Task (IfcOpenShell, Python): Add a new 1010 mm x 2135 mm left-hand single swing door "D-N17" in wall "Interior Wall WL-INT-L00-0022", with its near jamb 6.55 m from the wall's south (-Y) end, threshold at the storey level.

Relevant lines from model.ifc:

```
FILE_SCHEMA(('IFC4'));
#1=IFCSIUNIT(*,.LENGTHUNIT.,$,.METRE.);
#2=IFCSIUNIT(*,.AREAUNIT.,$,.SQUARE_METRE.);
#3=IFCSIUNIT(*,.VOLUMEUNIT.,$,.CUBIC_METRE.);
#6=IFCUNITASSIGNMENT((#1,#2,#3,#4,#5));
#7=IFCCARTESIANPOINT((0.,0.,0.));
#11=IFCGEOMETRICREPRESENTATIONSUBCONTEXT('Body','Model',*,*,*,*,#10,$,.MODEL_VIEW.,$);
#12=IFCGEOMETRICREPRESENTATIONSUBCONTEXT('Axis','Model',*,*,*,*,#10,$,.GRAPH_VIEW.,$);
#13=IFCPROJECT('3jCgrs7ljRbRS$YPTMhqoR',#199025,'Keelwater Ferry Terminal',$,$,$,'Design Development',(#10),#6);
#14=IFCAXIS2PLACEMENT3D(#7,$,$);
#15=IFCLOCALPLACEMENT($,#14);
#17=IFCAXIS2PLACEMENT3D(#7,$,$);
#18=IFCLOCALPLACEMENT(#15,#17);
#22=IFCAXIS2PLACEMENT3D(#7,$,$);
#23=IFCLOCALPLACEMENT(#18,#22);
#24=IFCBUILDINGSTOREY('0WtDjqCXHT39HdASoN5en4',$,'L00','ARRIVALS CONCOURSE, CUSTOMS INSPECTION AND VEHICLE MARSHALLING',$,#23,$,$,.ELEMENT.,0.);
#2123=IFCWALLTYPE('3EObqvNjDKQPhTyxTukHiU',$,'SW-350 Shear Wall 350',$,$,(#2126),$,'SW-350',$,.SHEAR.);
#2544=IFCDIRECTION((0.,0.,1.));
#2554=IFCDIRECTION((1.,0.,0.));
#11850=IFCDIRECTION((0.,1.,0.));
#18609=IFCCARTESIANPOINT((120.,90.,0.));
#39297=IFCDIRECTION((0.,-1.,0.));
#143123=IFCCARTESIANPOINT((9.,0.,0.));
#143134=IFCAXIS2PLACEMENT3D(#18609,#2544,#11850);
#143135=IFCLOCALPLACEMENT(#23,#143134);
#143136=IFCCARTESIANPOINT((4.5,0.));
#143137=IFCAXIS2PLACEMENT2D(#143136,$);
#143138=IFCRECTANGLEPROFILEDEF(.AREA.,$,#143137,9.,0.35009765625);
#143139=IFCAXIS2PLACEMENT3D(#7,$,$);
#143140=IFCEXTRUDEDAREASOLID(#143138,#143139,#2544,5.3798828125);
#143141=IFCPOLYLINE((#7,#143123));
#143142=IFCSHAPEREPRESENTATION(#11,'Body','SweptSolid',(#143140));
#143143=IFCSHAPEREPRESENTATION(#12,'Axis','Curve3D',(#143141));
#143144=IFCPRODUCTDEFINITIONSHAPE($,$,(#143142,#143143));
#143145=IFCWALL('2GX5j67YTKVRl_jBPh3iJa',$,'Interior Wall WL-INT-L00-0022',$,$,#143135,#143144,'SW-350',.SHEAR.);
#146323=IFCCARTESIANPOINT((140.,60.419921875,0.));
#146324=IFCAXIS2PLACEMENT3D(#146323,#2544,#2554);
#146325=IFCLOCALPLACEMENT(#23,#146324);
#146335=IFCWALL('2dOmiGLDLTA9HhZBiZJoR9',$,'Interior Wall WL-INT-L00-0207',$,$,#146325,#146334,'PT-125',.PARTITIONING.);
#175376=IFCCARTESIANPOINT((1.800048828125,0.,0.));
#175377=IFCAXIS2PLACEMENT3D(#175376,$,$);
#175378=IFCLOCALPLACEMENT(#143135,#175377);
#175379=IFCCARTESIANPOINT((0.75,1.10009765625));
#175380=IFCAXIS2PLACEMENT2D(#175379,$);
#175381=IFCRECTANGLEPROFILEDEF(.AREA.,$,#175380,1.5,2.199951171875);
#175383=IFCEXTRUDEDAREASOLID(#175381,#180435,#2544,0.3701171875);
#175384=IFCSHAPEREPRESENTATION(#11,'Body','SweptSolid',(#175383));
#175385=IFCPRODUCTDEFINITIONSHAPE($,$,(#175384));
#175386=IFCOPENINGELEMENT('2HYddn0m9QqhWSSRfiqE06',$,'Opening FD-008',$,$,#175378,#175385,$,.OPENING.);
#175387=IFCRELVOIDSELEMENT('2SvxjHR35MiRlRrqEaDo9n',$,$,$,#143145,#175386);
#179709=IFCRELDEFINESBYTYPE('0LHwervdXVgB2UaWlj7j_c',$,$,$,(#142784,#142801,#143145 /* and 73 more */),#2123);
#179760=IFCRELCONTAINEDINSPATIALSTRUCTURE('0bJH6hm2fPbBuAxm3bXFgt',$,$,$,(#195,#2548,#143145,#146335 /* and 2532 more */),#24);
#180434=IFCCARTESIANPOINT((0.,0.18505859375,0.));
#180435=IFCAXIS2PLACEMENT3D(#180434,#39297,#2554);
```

```python
import numpy as np
import ifcopenshell
import ifcopenshell.api.feature
import ifcopenshell.api.geometry
import ifcopenshell.api.root
import ifcopenshell.api.spatial
import ifcopenshell.geom
import ifcopenshell.util.element
import ifcopenshell.util.placement
import ifcopenshell.util.representation
import ifcopenshell.util.shape
import ifcopenshell.util.unit

model = ifcopenshell.open("model.ifc")
unit_scale = ifcopenshell.util.unit.calculate_unit_scale(model)
settings = ifcopenshell.geom.settings()


def volume(element):
    """Net volume in cubic metres, openings subtracted."""
    shape = ifcopenshell.geom.create_shape(settings, element)
    return ifcopenshell.util.shape.get_volume(shape.geometry)


wall = model.by_guid("2GX5j67YTKVRl_jBPh3iJa")
storey = ifcopenshell.util.element.get_container(wall, ifc_class="IfcBuildingStorey")
context = ifcopenshell.util.representation.get_context(model, "Model", "Body", "MODEL_VIEW")
before = volume(wall)

width, height, from_end, sill = 1.01, 2.135, 6.55, 0.0  # metres

# The wall runs along its own X axis, and the end named is its -X end.
wall_shape = ifcopenshell.geom.create_shape(settings, wall)
x, y, z = ifcopenshell.util.shape.get_vertices(wall_shape.geometry).T
start = x.min() + from_end
face, thickness = float(y.min()), float(y.max() - y.min())
wall_matrix = ifcopenshell.util.placement.get_local_placement(wall.ObjectPlacement)
level = ifcopenshell.util.placement.get_local_placement(storey.ObjectPlacement)[2, 3]


def in_wall(x, y):
    """Placement at x, y metres in the wall's axes, at sill height."""
    matrix = wall_matrix.copy()
    matrix[:, 3] = wall_matrix @ np.array([x / unit_scale, y / unit_scale, 0.0, 1.0])
    matrix[2, 3] = level + sill / unit_scale
    return matrix


# Opening: a box that overshoots both wall faces by 50 mm.
opening = ifcopenshell.api.root.create_entity(model, ifc_class="IfcOpeningElement", predefined_type="OPENING")
box = ifcopenshell.api.geometry.add_wall_representation(
    model, context=context, length=width, height=height, thickness=thickness + 0.1
)
ifcopenshell.api.geometry.assign_representation(model, product=opening, representation=box)
ifcopenshell.api.geometry.edit_object_placement(model, product=opening, matrix=in_wall(start, face - 0.05), is_si=False)
ifcopenshell.api.feature.add_feature(model, feature=opening, element=wall)

door = ifcopenshell.api.root.create_entity(model, ifc_class="IfcDoor", name="D-N17", predefined_type="DOOR")
door.OverallWidth, door.OverallHeight = width / unit_scale, height / unit_scale
door.OperationType = "SINGLE_SWING_LEFT"
body = ifcopenshell.api.geometry.add_door_representation(
    model,
    context=context,
    overall_width=door.OverallWidth,
    overall_height=door.OverallHeight,
    operation_type="SINGLE_SWING_LEFT",
    lining_properties={"LiningDepth": thickness / unit_scale, "ThresholdDepth": thickness / unit_scale},
)
ifcopenshell.api.geometry.assign_representation(model, product=door, representation=body)
ifcopenshell.api.spatial.assign_container(model, products=[door], relating_structure=storey)
ifcopenshell.api.feature.add_filling(model, opening=opening, element=door)

# The lining spans the wall, so the door starts at the wall face.
ifcopenshell.api.geometry.edit_object_placement(model, product=door, matrix=in_wall(start, face), is_si=False)

after = volume(wall)

print(f"wall volume {before:.3f} -> {after:.3f} m3")

model.write("model_updated.ifc")
```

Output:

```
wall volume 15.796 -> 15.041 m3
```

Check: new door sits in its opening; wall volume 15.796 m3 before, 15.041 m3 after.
